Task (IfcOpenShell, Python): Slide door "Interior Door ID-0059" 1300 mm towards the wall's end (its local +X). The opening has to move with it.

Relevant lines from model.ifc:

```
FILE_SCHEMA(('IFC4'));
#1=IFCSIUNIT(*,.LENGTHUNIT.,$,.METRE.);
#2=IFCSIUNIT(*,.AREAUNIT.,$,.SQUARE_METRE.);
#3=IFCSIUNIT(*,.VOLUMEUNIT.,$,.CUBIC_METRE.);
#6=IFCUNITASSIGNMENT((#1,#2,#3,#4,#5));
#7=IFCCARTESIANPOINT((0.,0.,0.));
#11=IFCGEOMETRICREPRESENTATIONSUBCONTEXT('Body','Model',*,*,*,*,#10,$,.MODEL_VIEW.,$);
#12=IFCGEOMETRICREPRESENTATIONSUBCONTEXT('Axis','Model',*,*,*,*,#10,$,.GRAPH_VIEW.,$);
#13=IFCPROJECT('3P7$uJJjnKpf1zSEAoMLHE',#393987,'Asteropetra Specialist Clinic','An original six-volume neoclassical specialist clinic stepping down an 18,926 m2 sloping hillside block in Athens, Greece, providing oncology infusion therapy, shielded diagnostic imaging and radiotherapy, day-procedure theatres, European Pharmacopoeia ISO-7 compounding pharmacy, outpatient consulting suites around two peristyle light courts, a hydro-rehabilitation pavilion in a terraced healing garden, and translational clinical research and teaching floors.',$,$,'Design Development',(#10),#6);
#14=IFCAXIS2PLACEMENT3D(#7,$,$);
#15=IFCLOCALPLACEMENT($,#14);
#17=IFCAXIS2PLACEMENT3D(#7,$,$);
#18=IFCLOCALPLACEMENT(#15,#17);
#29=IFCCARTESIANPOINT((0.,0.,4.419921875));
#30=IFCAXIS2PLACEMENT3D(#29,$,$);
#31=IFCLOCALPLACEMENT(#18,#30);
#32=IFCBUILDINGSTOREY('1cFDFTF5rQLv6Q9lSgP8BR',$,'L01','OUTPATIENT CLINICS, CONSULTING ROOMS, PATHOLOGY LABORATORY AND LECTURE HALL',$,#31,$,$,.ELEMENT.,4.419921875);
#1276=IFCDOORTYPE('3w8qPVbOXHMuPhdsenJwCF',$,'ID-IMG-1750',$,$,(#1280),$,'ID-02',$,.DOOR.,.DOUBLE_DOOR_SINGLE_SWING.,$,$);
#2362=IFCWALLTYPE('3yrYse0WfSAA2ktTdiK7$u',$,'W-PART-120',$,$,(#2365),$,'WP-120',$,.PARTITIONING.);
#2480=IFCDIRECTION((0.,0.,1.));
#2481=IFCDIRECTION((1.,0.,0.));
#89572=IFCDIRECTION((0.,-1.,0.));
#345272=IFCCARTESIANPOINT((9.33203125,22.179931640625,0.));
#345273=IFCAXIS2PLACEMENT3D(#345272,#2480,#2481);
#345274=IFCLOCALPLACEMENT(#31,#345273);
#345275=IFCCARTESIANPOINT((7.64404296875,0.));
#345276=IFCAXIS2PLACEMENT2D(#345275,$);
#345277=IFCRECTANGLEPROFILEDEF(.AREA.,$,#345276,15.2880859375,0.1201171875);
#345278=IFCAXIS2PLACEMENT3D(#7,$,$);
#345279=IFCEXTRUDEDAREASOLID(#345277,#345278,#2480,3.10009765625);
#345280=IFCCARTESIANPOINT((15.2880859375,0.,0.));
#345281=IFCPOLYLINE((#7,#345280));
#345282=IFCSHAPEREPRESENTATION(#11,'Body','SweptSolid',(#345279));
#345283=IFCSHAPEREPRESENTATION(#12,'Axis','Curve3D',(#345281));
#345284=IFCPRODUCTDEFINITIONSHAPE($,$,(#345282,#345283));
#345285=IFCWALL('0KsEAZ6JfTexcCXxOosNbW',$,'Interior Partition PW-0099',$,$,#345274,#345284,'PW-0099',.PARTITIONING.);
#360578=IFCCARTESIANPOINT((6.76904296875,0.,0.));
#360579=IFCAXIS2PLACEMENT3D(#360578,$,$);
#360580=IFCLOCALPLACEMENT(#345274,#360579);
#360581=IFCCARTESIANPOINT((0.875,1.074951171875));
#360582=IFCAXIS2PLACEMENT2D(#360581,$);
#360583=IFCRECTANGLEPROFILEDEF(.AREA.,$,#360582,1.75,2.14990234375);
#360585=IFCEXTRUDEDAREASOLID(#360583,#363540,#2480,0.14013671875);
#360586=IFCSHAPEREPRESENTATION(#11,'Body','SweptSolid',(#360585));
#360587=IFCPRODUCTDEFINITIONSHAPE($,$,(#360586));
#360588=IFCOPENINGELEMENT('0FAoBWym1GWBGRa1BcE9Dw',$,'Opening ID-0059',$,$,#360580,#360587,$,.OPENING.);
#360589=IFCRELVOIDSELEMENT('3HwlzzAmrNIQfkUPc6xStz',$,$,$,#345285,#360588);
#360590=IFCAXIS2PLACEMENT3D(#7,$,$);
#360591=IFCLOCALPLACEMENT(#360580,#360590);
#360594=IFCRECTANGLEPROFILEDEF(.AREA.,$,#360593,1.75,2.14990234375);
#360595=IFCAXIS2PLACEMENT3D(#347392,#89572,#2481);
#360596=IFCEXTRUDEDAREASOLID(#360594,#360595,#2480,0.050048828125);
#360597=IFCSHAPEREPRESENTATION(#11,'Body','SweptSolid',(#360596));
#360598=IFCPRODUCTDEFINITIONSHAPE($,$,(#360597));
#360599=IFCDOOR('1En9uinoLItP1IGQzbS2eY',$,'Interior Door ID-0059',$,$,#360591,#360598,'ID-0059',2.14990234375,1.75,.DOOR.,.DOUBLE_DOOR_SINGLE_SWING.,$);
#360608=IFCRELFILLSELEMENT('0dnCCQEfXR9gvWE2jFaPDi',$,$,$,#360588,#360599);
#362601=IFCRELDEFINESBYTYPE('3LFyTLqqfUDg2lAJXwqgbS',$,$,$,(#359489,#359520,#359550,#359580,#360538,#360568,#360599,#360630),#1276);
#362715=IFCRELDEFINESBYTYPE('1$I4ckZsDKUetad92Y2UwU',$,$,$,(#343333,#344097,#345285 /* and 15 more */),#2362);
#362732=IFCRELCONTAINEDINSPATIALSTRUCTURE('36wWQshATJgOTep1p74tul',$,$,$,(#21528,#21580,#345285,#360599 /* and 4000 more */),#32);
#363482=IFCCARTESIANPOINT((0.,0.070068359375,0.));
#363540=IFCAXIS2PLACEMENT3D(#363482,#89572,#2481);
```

```python
import ifcopenshell
import ifcopenshell.api.geometry
import ifcopenshell.util.placement
import ifcopenshell.util.unit

model = ifcopenshell.open("model.ifc")
unit_scale = ifcopenshell.util.unit.calculate_unit_scale(model)

door = model.by_guid("1En9uinoLItP1IGQzbS2eY")
opening = door.FillsVoids[0].RelatingOpeningElement
wall = opening.VoidsElements[0].RelatingBuildingElement

wall_matrix = ifcopenshell.util.placement.get_local_placement(wall.ObjectPlacement)
shift = wall_matrix[:3, 0] * 1.3 / unit_scale
before = ifcopenshell.util.placement.get_local_placement(door.ObjectPlacement)[:3, 3].copy()

# The door is placed relative to its opening, so it follows when the opening moves.
matrix = ifcopenshell.util.placement.get_local_placement(opening.ObjectPlacement)
matrix[:3, 3] += shift
ifcopenshell.api.geometry.edit_object_placement(
    model, product=opening, matrix=matrix, is_si=False, should_transform_children=True
)

after = ifcopenshell.util.placement.get_local_placement(door.ObjectPlacement)[:3, 3]
print("door moved by", (after - before).round(3) + 0.0)

model.write("model_edited.ifc")
```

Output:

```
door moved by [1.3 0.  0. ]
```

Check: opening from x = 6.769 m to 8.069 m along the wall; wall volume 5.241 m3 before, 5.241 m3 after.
